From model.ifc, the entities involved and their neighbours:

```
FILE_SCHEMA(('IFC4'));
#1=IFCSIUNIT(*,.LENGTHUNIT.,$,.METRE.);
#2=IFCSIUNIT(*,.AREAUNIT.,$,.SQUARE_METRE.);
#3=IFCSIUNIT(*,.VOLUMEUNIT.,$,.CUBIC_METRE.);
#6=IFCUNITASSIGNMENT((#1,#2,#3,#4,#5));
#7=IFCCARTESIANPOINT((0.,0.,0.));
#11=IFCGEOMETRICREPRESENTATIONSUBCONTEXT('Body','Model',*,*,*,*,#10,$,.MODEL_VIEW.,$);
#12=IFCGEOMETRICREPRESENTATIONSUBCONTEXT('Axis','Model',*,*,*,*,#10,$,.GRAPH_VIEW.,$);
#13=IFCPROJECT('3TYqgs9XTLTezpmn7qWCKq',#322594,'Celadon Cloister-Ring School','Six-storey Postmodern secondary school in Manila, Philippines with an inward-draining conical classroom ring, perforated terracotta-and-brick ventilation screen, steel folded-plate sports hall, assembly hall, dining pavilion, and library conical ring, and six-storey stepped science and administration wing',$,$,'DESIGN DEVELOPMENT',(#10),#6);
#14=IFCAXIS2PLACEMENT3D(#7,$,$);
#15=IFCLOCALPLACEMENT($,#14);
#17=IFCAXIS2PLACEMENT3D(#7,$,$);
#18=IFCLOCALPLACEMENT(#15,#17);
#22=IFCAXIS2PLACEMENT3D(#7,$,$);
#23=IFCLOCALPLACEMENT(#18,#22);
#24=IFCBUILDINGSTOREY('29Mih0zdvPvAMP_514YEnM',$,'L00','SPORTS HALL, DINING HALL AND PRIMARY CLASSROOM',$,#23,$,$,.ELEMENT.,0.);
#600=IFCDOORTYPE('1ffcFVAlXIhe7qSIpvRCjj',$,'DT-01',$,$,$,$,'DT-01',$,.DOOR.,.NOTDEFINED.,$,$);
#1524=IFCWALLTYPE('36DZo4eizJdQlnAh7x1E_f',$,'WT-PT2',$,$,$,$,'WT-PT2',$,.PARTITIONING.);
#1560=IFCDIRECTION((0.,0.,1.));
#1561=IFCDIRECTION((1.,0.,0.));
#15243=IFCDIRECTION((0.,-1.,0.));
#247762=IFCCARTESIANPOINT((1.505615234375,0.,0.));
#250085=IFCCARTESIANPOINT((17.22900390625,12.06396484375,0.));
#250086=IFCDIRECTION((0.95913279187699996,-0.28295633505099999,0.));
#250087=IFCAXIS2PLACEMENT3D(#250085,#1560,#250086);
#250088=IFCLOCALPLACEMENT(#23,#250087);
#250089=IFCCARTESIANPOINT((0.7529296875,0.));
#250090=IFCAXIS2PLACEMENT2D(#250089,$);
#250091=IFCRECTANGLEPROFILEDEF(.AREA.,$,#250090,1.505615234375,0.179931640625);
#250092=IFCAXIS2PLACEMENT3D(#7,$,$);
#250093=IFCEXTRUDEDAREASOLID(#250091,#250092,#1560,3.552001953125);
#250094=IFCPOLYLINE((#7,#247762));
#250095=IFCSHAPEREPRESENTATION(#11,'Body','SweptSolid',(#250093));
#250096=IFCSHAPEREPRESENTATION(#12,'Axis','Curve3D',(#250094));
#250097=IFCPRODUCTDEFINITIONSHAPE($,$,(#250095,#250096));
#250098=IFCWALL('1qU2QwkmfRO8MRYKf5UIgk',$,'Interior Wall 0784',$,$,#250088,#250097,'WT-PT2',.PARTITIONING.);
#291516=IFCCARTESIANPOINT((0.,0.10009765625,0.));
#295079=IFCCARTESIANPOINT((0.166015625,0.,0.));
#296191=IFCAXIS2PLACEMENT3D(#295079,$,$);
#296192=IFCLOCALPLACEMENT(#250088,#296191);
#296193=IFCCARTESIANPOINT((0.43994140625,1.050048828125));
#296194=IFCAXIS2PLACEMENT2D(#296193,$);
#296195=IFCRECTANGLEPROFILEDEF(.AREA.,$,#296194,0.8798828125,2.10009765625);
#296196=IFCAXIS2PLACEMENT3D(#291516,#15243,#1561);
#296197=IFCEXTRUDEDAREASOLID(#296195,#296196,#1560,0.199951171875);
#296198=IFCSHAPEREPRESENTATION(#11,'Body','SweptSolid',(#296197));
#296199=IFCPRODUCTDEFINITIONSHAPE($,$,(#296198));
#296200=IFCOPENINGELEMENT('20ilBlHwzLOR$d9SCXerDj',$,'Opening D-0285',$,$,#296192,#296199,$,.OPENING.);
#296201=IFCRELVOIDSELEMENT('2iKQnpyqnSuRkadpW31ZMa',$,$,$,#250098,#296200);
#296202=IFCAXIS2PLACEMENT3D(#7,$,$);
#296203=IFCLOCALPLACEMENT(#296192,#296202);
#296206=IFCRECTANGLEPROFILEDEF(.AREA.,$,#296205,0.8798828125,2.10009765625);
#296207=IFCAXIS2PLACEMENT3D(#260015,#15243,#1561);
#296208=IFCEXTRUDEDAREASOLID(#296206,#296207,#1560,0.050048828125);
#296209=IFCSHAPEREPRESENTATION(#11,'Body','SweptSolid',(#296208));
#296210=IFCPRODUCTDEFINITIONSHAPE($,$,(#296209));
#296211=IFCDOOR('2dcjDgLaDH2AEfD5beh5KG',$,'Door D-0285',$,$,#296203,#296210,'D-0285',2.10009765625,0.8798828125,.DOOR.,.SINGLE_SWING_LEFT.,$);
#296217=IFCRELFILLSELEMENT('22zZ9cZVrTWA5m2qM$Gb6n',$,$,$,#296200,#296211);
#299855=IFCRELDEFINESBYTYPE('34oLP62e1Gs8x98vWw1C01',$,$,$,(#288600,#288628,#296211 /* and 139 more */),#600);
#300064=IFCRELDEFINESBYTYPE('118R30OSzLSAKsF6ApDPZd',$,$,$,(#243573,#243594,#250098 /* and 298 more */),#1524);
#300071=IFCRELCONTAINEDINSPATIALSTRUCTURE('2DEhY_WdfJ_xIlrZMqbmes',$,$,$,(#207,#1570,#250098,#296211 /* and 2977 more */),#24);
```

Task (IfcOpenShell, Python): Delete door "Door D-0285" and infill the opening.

```python
import ifcopenshell
import ifcopenshell.api.feature
import ifcopenshell.api.root
import ifcopenshell.geom
import ifcopenshell.util.shape

model = ifcopenshell.open("model.ifc")
settings = ifcopenshell.geom.settings()


def volume(element):
    """Net volume in cubic metres, openings subtracted."""
    shape = ifcopenshell.geom.create_shape(settings, element)
    return ifcopenshell.util.shape.get_volume(shape.geometry)


door = model.by_guid("2dcjDgLaDH2AEfD5beh5KG")
opening = door.FillsVoids[0].RelatingOpeningElement
wall = opening.VoidsElements[0].RelatingBuildingElement
before = volume(wall)

ifcopenshell.api.root.remove_product(model, product=door)
ifcopenshell.api.feature.remove_feature(model, feature=opening)

after = volume(wall)

print(f"wall volume {before:.3f} -> {after:.3f} m3")

model.write("model-out.ifc")
```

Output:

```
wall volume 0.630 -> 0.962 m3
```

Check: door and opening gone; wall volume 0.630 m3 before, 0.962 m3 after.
